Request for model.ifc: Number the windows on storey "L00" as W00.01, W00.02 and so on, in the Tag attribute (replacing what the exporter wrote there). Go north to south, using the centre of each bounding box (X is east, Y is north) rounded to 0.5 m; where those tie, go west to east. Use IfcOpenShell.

First a look at what the model holds.

```python
import ifcopenshell
import ifcopenshell.util.element
import ifcopenshell.util.placement

model = ifcopenshell.open("model.ifc")
print(model.schema)
storey = next(s for s in model.by_type("IfcBuildingStorey") if s.Name == "L00")
windows = [e for e in ifcopenshell.util.element.get_decomposition(storey) if e.is_a("IfcWindow")]
for e in sorted(windows, key=lambda e: e.id()):
    origin = ifcopenshell.util.placement.get_local_placement(e.ObjectPlacement)[:3, 3]
    print(e.id(), e.Tag, e.Name, origin.round(2) + 0.0, sep=" | ")
```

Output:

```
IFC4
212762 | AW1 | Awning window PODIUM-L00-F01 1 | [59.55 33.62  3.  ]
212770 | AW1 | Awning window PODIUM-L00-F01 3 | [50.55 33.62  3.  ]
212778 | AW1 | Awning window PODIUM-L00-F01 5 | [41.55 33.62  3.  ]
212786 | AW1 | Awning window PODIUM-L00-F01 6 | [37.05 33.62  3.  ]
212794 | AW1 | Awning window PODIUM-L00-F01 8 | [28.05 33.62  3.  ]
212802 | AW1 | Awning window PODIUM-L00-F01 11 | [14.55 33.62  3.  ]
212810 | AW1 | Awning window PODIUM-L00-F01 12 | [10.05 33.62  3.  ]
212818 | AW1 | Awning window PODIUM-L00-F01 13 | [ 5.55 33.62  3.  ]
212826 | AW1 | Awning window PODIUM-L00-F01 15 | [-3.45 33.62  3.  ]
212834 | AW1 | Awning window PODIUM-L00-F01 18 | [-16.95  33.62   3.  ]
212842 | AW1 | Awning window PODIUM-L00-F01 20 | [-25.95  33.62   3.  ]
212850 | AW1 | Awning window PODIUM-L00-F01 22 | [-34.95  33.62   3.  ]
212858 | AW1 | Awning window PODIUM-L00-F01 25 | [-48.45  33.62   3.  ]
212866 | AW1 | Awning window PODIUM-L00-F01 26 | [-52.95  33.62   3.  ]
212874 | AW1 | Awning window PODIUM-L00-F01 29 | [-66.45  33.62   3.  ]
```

```python
import ifcopenshell
import ifcopenshell.geom
import ifcopenshell.util.element
import ifcopenshell.util.shape

model = ifcopenshell.open("model.ifc")
settings = ifcopenshell.geom.settings()
settings.set("use-world-coords", True)


def centre(element):
    shape = ifcopenshell.geom.create_shape(settings, element)
    return ifcopenshell.util.shape.get_bbox_centroid(shape.geometry)


storey = next(s for s in model.by_type("IfcBuildingStorey") if s.Name == "L00")
windows = [e for e in ifcopenshell.util.element.get_decomposition(storey) if e.is_a("IfcWindow")]

# Insertion points can sit at a corner or the storey origin, so sort by the geometry (in metres).
centres = {e: centre(e) for e in windows}
windows.sort(key=lambda e: (-round(centres[e][1] / 0.5), centres[e][0]))

for i, e in enumerate(windows, start=1):
    number = f"W00.{i:02d}"
    e.Tag = number
    print(e.id(), number)

model.write("model_updated.ifc")
```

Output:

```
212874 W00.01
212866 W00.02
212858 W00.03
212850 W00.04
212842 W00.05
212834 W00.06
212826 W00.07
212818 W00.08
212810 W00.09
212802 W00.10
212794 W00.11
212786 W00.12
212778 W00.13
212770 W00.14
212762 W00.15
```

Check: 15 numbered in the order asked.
